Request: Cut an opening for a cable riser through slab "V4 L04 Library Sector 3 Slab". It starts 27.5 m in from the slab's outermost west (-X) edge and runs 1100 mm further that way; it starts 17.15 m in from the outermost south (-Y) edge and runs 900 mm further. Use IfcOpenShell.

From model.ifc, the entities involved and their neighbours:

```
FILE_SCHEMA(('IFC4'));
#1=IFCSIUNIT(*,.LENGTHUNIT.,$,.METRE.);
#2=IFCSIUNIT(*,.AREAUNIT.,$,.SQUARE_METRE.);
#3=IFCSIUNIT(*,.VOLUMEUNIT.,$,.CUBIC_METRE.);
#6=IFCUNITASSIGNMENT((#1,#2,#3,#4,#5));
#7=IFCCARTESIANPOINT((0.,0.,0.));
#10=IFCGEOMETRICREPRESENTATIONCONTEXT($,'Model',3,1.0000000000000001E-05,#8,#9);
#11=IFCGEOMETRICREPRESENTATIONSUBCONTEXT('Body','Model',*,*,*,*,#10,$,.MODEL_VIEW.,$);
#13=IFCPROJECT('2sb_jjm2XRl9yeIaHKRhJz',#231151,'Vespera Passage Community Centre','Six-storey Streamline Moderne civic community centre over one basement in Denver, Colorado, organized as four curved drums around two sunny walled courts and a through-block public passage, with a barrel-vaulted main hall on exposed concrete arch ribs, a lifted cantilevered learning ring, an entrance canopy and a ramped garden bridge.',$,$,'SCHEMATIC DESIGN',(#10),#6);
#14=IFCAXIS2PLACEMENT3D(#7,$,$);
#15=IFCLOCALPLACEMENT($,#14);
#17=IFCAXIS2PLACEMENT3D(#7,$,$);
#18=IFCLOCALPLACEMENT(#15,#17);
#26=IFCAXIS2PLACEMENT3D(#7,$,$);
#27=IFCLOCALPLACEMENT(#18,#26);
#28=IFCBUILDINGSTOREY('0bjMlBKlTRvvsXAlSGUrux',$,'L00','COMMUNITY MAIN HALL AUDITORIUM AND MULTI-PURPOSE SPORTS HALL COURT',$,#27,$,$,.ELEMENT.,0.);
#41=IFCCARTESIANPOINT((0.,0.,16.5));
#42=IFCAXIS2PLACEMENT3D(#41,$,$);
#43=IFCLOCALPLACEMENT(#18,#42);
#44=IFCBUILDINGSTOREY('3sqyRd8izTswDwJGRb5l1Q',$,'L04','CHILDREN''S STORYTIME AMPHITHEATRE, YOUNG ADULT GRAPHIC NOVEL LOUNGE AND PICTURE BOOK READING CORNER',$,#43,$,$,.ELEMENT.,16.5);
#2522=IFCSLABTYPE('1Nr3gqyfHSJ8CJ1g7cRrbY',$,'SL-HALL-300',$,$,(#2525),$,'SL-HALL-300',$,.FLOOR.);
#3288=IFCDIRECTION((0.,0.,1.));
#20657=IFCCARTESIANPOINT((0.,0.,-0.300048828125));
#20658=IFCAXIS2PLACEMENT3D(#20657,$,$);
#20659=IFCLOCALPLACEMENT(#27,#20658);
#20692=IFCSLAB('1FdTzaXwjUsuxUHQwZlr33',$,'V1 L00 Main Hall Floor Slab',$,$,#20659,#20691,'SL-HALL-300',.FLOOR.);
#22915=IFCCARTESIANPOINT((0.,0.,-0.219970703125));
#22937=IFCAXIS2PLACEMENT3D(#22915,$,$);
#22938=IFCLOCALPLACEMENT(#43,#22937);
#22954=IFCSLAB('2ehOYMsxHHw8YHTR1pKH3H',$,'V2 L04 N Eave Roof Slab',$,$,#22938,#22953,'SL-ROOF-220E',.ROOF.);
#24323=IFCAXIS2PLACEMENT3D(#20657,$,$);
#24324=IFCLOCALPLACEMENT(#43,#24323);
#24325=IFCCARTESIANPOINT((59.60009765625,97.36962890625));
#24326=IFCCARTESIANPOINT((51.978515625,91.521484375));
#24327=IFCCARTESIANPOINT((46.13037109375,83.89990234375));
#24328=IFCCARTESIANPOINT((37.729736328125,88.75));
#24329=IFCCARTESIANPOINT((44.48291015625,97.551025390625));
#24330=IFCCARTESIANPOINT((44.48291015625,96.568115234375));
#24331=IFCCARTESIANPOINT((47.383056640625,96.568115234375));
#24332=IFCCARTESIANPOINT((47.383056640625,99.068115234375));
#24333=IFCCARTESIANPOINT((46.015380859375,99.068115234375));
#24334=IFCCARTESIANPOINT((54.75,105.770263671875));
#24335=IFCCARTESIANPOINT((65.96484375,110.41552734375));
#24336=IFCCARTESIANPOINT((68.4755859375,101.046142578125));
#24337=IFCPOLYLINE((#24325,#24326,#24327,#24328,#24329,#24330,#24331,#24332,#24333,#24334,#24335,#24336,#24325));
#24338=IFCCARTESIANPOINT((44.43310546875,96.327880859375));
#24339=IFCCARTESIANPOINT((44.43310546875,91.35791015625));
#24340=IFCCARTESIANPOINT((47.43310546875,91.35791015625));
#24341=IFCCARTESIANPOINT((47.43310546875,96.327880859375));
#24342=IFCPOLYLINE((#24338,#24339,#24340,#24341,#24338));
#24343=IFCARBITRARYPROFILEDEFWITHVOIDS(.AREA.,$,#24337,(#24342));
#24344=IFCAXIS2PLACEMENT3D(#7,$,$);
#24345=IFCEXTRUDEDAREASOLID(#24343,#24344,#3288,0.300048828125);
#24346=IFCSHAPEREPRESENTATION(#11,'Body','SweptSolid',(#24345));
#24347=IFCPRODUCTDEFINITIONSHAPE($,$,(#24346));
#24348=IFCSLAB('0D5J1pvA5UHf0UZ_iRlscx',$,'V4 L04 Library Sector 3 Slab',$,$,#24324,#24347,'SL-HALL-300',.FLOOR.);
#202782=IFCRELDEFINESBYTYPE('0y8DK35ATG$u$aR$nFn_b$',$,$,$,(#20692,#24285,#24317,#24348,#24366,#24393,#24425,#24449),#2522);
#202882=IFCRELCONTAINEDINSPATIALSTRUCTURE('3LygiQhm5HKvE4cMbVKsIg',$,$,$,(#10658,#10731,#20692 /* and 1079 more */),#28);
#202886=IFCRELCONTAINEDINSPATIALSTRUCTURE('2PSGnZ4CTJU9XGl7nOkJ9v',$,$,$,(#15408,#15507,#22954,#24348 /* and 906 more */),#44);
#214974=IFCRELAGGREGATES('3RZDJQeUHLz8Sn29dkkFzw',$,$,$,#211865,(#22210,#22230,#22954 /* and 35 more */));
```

```python
import numpy as np
import ifcopenshell
import ifcopenshell.api.feature
import ifcopenshell.api.geometry
import ifcopenshell.api.root
import ifcopenshell.geom
import ifcopenshell.util.placement
import ifcopenshell.util.representation
import ifcopenshell.util.shape
import ifcopenshell.util.unit

model = ifcopenshell.open("model.ifc")
unit_scale = ifcopenshell.util.unit.calculate_unit_scale(model)
settings = ifcopenshell.geom.settings()


def volume(element):
    """Net volume in cubic metres, openings subtracted."""
    shape = ifcopenshell.geom.create_shape(settings, element)
    return ifcopenshell.util.shape.get_volume(shape.geometry)


slab = model.by_id(24348)
before = volume(slab)

# Extent in the slab's own axes, in metres. The edges named are its -X and -Y sides.
slab_shape = ifcopenshell.geom.create_shape(settings, slab)
vertices = ifcopenshell.util.shape.get_vertices(slab_shape.geometry)
x_min, y_min, bottom = vertices.min(axis=0)
top = vertices[:, 2].max()

opening = ifcopenshell.api.root.create_entity(model, ifc_class="IfcOpeningElement", name="Cable riser opening", predefined_type="OPENING")
context = ifcopenshell.util.representation.get_context(model, "Model", "Body", "MODEL_VIEW")
width, depth = 1.1, 0.9
outline = [(0.0, 0.0), (width, 0.0), (width, depth), (0.0, depth), (0.0, 0.0)]
# Overshoot both faces by 50 mm so the cut is clean.
shape = ifcopenshell.api.geometry.add_slab_representation(
    model, context=context, depth=top - bottom + 0.1, polyline=outline
)
ifcopenshell.api.geometry.assign_representation(model, product=opening, representation=shape)

matrix = ifcopenshell.util.placement.get_local_placement(slab.ObjectPlacement)
matrix[:, 3] = matrix @ np.append(np.array([x_min + 27.5, y_min + 17.15, bottom - 0.05]) / unit_scale, 1.0)
ifcopenshell.api.geometry.edit_object_placement(model, product=opening, matrix=matrix, is_si=False)
ifcopenshell.api.feature.add_feature(model, feature=opening, element=slab)

after = volume(slab)

print(f"slab volume {before:.3f} -> {after:.3f} m3")

model.write("model_updated.ifc")
```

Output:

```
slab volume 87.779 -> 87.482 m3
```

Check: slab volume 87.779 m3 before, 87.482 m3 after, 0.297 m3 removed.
